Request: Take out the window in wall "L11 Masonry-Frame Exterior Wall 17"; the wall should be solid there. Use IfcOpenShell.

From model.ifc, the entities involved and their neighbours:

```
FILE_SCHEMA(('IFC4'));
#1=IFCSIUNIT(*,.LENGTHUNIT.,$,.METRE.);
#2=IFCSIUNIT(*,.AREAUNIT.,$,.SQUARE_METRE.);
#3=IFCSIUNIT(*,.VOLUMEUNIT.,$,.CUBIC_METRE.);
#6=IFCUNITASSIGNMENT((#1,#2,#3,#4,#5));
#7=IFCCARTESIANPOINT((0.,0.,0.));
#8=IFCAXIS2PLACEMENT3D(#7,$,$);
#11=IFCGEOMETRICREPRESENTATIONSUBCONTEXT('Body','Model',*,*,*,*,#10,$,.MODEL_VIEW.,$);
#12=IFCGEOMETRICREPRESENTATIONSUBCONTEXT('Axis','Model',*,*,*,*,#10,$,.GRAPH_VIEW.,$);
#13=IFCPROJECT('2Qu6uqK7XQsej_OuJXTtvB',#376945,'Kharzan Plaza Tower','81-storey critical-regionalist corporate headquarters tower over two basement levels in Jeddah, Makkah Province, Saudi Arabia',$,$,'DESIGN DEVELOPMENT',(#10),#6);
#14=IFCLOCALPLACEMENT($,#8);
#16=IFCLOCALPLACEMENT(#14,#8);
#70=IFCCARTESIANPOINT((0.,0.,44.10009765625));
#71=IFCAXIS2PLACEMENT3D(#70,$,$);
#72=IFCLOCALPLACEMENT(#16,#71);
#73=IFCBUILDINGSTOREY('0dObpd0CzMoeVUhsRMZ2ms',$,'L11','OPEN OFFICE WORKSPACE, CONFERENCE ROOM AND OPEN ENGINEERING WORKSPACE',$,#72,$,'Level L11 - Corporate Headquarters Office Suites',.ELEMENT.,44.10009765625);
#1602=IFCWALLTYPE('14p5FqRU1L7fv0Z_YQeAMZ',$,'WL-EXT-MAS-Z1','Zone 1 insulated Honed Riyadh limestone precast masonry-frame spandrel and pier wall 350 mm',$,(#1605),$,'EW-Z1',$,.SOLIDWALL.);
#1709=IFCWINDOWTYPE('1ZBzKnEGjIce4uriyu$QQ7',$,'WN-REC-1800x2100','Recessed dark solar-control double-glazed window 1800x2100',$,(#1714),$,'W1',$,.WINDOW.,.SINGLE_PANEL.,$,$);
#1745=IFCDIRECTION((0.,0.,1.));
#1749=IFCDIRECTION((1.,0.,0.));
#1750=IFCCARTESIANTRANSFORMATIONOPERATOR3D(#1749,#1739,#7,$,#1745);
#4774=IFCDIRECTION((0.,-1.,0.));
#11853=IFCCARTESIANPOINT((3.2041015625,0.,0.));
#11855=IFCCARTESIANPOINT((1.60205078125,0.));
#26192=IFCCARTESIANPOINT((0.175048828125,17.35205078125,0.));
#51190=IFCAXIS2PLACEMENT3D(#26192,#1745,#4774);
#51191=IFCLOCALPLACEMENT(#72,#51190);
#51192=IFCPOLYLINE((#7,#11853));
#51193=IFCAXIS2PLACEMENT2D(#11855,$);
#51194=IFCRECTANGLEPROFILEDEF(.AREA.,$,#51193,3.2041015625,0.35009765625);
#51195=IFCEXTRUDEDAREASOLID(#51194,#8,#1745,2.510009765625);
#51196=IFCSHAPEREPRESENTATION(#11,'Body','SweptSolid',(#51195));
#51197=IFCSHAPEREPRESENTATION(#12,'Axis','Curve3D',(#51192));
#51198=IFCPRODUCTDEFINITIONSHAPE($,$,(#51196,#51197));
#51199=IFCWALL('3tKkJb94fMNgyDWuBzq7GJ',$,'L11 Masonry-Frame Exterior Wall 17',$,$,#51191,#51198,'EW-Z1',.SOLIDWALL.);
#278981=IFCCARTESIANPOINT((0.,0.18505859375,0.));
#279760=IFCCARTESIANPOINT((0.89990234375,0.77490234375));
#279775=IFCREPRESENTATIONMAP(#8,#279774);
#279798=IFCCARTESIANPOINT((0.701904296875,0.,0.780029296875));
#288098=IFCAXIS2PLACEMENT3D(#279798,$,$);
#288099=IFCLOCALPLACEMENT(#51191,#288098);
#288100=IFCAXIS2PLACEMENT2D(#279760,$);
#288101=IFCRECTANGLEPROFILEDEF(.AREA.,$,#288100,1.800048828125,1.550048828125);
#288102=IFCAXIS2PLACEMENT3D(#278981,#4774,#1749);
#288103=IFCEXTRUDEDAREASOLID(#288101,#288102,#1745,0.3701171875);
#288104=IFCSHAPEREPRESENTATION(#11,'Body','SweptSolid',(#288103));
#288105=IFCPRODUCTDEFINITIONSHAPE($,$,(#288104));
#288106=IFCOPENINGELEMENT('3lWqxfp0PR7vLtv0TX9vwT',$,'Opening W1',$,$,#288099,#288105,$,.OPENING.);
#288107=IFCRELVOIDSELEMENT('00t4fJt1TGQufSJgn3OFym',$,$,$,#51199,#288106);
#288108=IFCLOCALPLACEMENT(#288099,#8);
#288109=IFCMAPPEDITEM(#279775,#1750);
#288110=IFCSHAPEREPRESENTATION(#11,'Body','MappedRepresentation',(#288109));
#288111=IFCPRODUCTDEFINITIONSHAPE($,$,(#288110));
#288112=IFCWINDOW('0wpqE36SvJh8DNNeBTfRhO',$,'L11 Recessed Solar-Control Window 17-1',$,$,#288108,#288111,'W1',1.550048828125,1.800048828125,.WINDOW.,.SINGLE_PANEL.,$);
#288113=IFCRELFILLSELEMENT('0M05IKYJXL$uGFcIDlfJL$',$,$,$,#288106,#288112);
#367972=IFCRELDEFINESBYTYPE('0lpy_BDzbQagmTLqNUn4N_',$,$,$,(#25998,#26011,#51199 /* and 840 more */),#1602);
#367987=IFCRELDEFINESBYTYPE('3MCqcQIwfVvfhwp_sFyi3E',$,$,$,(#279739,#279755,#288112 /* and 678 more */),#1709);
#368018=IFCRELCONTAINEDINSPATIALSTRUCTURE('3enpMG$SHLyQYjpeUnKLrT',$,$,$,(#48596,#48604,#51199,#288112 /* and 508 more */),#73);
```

```python
import ifcopenshell
import ifcopenshell.api.feature
import ifcopenshell.api.root
import ifcopenshell.geom
import ifcopenshell.util.shape

model = ifcopenshell.open("model.ifc")
settings = ifcopenshell.geom.settings()


def volume(element):
    """Net volume in cubic metres, openings subtracted."""
    shape = ifcopenshell.geom.create_shape(settings, element)
    return ifcopenshell.util.shape.get_volume(shape.geometry)


window = model.by_id(288112)
opening = window.FillsVoids[0].RelatingOpeningElement
wall = opening.VoidsElements[0].RelatingBuildingElement
before = volume(wall)

ifcopenshell.api.root.remove_product(model, product=window)
ifcopenshell.api.feature.remove_feature(model, feature=opening)

after = volume(wall)

print(f"wall volume {before:.3f} -> {after:.3f} m3")

model.write("model_edited.ifc")
```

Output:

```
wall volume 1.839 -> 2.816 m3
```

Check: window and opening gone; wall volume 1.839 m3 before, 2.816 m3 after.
